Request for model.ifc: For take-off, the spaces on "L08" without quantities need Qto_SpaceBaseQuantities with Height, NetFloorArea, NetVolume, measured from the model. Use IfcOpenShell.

First a look at what the model holds.

```python
import ifcopenshell
import ifcopenshell.util.element
import ifcopenshell.util.unit

model = ifcopenshell.open("model.ifc")
print(model.schema)
for unit_type in ("LENGTHUNIT", "AREAUNIT", "VOLUMEUNIT"):
    print(unit_type, ifcopenshell.util.unit.calculate_unit_scale(model, unit_type))
storey = next(s for s in model.by_type("IfcBuildingStorey") if s.Name == "L08")
spaces = [e for e in ifcopenshell.util.element.get_decomposition(storey) if e.is_a("IfcSpace")]
for e in sorted(spaces, key=lambda e: e.id()):
    print(e.id(), e.is_a(), e.Name, list(ifcopenshell.util.element.get_psets(e, qtos_only=True)), sep=" | ")
```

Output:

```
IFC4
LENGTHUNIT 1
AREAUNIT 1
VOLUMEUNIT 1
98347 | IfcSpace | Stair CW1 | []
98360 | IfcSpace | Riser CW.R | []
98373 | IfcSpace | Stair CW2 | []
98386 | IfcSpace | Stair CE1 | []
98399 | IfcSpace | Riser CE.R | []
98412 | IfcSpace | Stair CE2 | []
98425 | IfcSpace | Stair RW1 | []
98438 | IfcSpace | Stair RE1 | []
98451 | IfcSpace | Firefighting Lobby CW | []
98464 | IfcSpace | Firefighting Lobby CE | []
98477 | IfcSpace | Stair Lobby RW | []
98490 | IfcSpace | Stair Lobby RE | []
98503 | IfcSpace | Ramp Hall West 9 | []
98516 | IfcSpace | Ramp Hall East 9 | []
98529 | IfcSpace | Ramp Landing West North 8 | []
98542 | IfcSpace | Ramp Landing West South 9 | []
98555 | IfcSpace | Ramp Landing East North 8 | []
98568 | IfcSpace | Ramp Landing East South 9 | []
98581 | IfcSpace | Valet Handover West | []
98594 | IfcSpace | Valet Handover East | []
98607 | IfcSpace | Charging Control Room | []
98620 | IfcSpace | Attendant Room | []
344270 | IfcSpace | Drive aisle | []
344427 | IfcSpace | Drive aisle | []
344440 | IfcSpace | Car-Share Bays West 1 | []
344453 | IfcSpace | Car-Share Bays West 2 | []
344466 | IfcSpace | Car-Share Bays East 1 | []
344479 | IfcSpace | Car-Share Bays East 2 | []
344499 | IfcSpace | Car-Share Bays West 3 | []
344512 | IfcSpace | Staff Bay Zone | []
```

```python
import ifcopenshell
import ifcopenshell.api.pset
import ifcopenshell.geom
import ifcopenshell.util.element
import ifcopenshell.util.shape
import ifcopenshell.util.unit

model = ifcopenshell.open("model.ifc")
unit_scale = ifcopenshell.util.unit.calculate_unit_scale(model)
area_scale = ifcopenshell.util.unit.calculate_unit_scale(model, "AREAUNIT")
volume_scale = ifcopenshell.util.unit.calculate_unit_scale(model, "VOLUMEUNIT")
settings = ifcopenshell.geom.settings()

storey = next(s for s in model.by_type("IfcBuildingStorey") if s.Name == "L08")
spaces = [e for e in ifcopenshell.util.element.get_decomposition(storey) if e.is_a("IfcSpace")]

for e in sorted(spaces, key=lambda e: e.id()):
    if ifcopenshell.util.element.get_psets(e, qtos_only=True, should_inherit=False):
        continue
    # Geometry comes back in metres, in the element's own axes.
    shape = ifcopenshell.geom.create_shape(settings, e)
    values = {
        "Height": ifcopenshell.util.shape.get_z(shape.geometry) / unit_scale,
        "NetFloorArea": ifcopenshell.util.shape.get_footprint_area(shape.geometry) / area_scale,
        "NetVolume": ifcopenshell.util.shape.get_volume(shape.geometry) / volume_scale,
    }
    qto = ifcopenshell.api.pset.add_qto(model, product=e, name="Qto_SpaceBaseQuantities")
    ifcopenshell.api.pset.edit_qto(model, qto=qto, properties=values)
    print(e.id(), {k: round(v, 3) for k, v in values.items()})

model.write("model_rev.ifc")
```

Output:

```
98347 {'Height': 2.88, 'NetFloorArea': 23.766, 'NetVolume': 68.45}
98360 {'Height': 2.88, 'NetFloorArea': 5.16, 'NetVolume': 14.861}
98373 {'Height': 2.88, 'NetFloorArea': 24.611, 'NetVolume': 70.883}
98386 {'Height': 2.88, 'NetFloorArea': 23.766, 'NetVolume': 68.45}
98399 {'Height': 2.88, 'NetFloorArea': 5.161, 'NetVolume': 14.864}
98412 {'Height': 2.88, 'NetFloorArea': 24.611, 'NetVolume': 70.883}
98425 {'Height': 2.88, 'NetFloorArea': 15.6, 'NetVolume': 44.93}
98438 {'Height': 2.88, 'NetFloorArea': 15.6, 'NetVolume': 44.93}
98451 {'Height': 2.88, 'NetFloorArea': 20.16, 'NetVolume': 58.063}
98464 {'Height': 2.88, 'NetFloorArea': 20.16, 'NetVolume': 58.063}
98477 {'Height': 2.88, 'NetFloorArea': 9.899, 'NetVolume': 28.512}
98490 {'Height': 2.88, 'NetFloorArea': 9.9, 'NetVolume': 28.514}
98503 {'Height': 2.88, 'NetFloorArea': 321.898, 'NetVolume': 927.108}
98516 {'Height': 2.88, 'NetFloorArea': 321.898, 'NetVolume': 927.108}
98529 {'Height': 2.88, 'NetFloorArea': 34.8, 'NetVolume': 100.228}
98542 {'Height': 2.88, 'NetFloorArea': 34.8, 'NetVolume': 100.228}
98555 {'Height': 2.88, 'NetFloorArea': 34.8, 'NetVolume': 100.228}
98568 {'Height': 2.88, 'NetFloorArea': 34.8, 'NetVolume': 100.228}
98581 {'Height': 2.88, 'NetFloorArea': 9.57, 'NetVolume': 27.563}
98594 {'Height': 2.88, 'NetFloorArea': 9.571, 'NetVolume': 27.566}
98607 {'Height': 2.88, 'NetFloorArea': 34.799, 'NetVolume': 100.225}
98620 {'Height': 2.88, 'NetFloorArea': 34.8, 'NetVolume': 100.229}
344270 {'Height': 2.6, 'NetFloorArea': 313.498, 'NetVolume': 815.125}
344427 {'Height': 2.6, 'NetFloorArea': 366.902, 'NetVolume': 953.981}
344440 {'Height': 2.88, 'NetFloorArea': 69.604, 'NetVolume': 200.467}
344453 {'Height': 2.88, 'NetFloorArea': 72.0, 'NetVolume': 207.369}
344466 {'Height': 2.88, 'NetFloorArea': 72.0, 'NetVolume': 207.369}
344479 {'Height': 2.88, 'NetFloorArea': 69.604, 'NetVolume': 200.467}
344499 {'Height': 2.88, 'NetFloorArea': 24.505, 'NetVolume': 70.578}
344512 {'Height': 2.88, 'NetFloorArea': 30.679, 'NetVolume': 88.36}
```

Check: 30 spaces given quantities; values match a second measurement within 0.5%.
